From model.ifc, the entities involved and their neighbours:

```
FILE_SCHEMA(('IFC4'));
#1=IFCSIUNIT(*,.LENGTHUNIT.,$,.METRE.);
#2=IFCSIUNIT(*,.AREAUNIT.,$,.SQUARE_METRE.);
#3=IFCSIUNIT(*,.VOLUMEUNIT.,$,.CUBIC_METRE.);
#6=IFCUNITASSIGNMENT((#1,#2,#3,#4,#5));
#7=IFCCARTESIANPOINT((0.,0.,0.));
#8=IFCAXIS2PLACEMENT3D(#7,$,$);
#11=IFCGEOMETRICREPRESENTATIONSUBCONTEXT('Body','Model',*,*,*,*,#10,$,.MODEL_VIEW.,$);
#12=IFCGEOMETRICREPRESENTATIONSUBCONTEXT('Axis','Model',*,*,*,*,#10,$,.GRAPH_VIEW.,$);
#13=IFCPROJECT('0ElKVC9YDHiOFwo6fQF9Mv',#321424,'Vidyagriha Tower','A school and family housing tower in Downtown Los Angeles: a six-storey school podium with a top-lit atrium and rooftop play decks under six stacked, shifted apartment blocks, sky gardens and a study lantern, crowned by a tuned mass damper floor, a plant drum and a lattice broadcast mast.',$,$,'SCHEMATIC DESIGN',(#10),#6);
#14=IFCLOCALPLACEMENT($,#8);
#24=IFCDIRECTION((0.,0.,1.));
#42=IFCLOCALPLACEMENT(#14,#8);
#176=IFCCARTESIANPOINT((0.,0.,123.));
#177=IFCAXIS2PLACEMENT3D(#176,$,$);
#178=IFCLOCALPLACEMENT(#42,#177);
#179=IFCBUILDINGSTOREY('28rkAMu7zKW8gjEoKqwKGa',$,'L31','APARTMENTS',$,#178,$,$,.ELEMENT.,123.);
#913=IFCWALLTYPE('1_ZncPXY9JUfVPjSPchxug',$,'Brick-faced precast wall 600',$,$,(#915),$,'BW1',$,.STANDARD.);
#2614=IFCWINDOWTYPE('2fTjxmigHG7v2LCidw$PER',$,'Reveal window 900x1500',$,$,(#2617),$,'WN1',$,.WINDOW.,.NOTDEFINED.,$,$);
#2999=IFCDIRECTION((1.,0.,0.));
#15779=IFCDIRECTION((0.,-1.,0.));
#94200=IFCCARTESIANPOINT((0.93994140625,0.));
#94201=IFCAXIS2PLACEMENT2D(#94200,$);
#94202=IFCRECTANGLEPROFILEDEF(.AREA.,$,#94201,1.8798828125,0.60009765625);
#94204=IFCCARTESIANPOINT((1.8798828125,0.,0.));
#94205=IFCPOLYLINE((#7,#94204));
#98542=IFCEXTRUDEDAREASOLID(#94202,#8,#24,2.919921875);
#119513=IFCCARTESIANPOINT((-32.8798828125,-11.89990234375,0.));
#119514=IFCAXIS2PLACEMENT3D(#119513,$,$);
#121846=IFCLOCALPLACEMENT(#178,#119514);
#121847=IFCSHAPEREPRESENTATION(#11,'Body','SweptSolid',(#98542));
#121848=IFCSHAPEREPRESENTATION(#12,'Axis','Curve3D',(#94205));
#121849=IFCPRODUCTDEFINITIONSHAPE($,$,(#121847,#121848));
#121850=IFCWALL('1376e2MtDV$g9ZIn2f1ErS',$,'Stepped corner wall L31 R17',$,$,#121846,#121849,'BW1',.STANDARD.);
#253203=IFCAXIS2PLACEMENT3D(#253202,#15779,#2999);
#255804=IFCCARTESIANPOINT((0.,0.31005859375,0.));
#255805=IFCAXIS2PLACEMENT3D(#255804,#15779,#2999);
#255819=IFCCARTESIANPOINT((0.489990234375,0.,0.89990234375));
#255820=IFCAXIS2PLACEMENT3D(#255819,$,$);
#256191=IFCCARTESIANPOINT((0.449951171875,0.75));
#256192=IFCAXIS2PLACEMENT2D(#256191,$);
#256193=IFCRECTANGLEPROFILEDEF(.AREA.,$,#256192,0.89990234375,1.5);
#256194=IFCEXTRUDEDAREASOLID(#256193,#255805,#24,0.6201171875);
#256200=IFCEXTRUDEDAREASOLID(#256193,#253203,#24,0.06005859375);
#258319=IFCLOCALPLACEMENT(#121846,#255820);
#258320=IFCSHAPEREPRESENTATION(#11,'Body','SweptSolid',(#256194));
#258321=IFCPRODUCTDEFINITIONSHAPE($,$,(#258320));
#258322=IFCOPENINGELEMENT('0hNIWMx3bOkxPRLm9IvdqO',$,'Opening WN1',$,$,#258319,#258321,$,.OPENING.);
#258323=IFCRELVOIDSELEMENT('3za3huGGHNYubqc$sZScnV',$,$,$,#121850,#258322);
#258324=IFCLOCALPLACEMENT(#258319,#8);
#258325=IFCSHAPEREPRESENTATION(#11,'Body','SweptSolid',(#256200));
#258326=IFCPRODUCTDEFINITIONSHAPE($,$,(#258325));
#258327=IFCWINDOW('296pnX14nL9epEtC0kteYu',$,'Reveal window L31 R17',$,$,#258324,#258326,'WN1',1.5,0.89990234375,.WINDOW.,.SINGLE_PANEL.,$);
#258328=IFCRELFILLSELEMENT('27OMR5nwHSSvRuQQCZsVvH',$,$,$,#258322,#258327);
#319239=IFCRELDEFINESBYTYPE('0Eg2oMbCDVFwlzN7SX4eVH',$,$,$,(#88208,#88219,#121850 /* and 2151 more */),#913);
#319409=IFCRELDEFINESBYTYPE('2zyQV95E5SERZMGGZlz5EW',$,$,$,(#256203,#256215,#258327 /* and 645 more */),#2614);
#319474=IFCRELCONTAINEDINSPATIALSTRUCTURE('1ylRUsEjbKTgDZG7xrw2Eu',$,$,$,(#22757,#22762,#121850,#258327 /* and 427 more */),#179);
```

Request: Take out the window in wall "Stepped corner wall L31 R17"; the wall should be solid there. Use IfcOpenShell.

```python
import ifcopenshell
import ifcopenshell.api.feature
import ifcopenshell.api.root
import ifcopenshell.geom
import ifcopenshell.util.shape

model = ifcopenshell.open("model.ifc")
settings = ifcopenshell.geom.settings()


def volume(element):
    """Net volume in cubic metres, openings subtracted."""
    shape = ifcopenshell.geom.create_shape(settings, element)
    return ifcopenshell.util.shape.get_volume(shape.geometry)


window = model.by_guid("296pnX14nL9epEtC0kteYu")
opening = window.FillsVoids[0].RelatingOpeningElement
wall = opening.VoidsElements[0].RelatingBuildingElement
before = volume(wall)

ifcopenshell.api.root.remove_product(model, product=window)
ifcopenshell.api.feature.remove_feature(model, feature=opening)

after = volume(wall)

print(f"wall volume {before:.3f} -> {after:.3f} m3")

model.write("model_updated.ifc")
```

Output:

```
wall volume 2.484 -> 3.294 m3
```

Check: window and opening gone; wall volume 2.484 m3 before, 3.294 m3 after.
